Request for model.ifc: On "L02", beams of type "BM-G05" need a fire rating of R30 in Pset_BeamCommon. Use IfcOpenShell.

First a look at what the model holds.

```python
import ifcopenshell
import ifcopenshell.util.element

model = ifcopenshell.open("model.ifc")
print(model.schema)
storey = next(s for s in model.by_type("IfcBuildingStorey") if s.Name == "L02")
beams = [e for e in ifcopenshell.util.element.get_decomposition(storey) if e.is_a("IfcBeam")]
seen = {}
for e in beams:
    element_type = ifcopenshell.util.element.get_type(e)
    key = (element_type.Name if element_type != e and element_type else None, ifcopenshell.util.element.get_pset(e, "Pset_BeamCommon", "FireRating"))
    seen[key] = seen.get(key, 0) + 1
for (name, value), count in sorted(seen.items(), key=str):
    print(count, "x", name, "|", value)
```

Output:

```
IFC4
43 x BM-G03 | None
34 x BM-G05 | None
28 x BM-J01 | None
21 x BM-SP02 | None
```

```python
import ifcopenshell
import ifcopenshell.api.pset
import ifcopenshell.util.element

model = ifcopenshell.open("model.ifc")

storey = next(s for s in model.by_type("IfcBuildingStorey") if s.Name == "L02")
beams = [e for e in ifcopenshell.util.element.get_decomposition(storey) if e.is_a("IfcBeam")]

count = 0
for e in beams:
    element_type = ifcopenshell.util.element.get_type(e)
    if element_type in (None, e) or element_type.Name != "BM-G05":
        continue
    # add_pset returns the element's existing set when there is one.
    pset = ifcopenshell.api.pset.add_pset(model, product=e, name="Pset_BeamCommon")
    ifcopenshell.api.pset.edit_pset(model, pset=pset, properties={"FireRating": "R30"})
    count += 1

print(count, "beams updated")

model.write("model_edited.ifc")
```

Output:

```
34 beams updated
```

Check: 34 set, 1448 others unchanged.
